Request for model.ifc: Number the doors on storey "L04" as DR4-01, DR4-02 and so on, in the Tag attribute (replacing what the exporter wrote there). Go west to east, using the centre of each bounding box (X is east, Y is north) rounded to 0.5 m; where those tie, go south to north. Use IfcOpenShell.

First a look at what the model holds.

```python
import ifcopenshell
import ifcopenshell.util.element
import ifcopenshell.util.placement

model = ifcopenshell.open("model.ifc")
print(model.schema)
storey = next(s for s in model.by_type("IfcBuildingStorey") if s.Name == "L04")
doors = [e for e in ifcopenshell.util.element.get_decomposition(storey) if e.is_a("IfcDoor")]
for e in sorted(doors, key=lambda e: e.id()):
    origin = ifcopenshell.util.placement.get_local_placement(e.ObjectPlacement)[:3, 3]
    print(e.id(), e.Tag, e.Name, origin.round(2) + 0.0, sep=" | ")
```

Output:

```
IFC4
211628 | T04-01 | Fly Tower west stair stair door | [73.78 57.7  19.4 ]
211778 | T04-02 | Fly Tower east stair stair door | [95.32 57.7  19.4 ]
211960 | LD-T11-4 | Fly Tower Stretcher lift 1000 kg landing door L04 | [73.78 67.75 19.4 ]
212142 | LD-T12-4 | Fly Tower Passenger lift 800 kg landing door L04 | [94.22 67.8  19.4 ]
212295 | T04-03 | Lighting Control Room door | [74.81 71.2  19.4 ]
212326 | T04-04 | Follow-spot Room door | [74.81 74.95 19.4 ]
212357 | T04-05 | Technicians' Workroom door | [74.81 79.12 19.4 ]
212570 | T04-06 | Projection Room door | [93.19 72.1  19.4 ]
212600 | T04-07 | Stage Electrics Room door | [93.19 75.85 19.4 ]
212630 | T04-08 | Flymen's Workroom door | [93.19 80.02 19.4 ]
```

```python
import ifcopenshell
import ifcopenshell.geom
import ifcopenshell.util.element
import ifcopenshell.util.shape

model = ifcopenshell.open("model.ifc")
settings = ifcopenshell.geom.settings()
settings.set("use-world-coords", True)


def centre(element):
    shape = ifcopenshell.geom.create_shape(settings, element)
    return ifcopenshell.util.shape.get_bbox_centroid(shape.geometry)


storey = next(s for s in model.by_type("IfcBuildingStorey") if s.Name == "L04")
doors = [e for e in ifcopenshell.util.element.get_decomposition(storey) if e.is_a("IfcDoor")]

# Insertion points can sit at a corner or the storey origin, so sort by the geometry (in metres).
centres = {e: centre(e) for e in doors}
doors.sort(key=lambda e: (round(centres[e][0] / 0.5), centres[e][1]))

for i, e in enumerate(doors, start=1):
    number = f"DR4-{i:02d}"
    e.Tag = number
    print(e.id(), number)

model.write("model_v2.ifc")
```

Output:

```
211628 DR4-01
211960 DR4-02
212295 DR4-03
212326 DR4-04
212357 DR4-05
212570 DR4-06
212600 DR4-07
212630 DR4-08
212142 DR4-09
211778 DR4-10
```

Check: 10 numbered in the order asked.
